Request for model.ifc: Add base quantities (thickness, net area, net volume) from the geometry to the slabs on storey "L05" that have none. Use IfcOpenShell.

First a look at what the model holds.

```python
import ifcopenshell
import ifcopenshell.util.element
import ifcopenshell.util.unit

model = ifcopenshell.open("model.ifc")
print(model.schema)
for unit_type in ("LENGTHUNIT", "AREAUNIT", "VOLUMEUNIT"):
    print(unit_type, ifcopenshell.util.unit.calculate_unit_scale(model, unit_type))
storey = next(s for s in model.by_type("IfcBuildingStorey") if s.Name == "L05")
slabs = [e for e in ifcopenshell.util.element.get_decomposition(storey) if e.is_a("IfcSlab")]
for e in sorted(slabs, key=lambda e: e.id()):
    print(e.id(), e.is_a(), e.Name, list(ifcopenshell.util.element.get_psets(e, qtos_only=True)), sep=" | ")
```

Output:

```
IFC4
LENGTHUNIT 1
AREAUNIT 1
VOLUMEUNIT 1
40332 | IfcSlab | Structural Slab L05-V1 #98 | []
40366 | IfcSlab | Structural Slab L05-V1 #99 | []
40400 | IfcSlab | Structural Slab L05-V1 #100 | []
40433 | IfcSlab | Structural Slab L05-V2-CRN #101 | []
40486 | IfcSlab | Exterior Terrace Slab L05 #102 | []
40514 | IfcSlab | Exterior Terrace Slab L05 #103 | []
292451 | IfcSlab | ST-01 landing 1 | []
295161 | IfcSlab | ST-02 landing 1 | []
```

```python
import ifcopenshell
import ifcopenshell.api.pset
import ifcopenshell.geom
import ifcopenshell.util.element
import ifcopenshell.util.shape
import ifcopenshell.util.unit

model = ifcopenshell.open("model.ifc")
unit_scale = ifcopenshell.util.unit.calculate_unit_scale(model)
area_scale = ifcopenshell.util.unit.calculate_unit_scale(model, "AREAUNIT")
volume_scale = ifcopenshell.util.unit.calculate_unit_scale(model, "VOLUMEUNIT")
settings = ifcopenshell.geom.settings()

storey = next(s for s in model.by_type("IfcBuildingStorey") if s.Name == "L05")
slabs = [e for e in ifcopenshell.util.element.get_decomposition(storey) if e.is_a("IfcSlab")]

for e in sorted(slabs, key=lambda e: e.id()):
    if ifcopenshell.util.element.get_psets(e, qtos_only=True, should_inherit=False):
        continue
    # Geometry comes back in metres, in the element's own axes.
    shape = ifcopenshell.geom.create_shape(settings, e)
    values = {
        "Width": ifcopenshell.util.shape.get_z(shape.geometry) / unit_scale,
        "NetArea": ifcopenshell.util.shape.get_footprint_area(shape.geometry) / area_scale,
        "NetVolume": ifcopenshell.util.shape.get_volume(shape.geometry) / volume_scale,
    }
    qto = ifcopenshell.api.pset.add_qto(model, product=e, name="Qto_SlabBaseQuantities")
    ifcopenshell.api.pset.edit_qto(model, qto=qto, properties=values)
    print(e.id(), {k: round(v, 3) for k, v in values.items()})

model.write("model_v2.ifc")
```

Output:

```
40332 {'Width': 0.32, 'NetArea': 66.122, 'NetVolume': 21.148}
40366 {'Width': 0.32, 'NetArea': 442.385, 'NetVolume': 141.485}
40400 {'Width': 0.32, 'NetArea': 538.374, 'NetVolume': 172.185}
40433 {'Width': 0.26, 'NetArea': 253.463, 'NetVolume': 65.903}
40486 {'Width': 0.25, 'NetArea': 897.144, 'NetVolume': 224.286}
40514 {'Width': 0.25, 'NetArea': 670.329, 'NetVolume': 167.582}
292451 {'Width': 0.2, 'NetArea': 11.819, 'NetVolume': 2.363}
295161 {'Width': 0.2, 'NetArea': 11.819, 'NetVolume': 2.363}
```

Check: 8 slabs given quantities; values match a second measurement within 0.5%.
